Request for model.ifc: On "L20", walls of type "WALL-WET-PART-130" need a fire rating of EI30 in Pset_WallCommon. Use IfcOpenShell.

First a look at what the model holds.

```python
import ifcopenshell
import ifcopenshell.util.element

model = ifcopenshell.open("model.ifc")
print(model.schema)
storey = next(s for s in model.by_type("IfcBuildingStorey") if s.Name == "L20")
walls = [e for e in ifcopenshell.util.element.get_decomposition(storey) if e.is_a("IfcWall")]
seen = {}
for e in walls:
    element_type = ifcopenshell.util.element.get_type(e)
    key = (element_type.Name if element_type != e and element_type else None, ifcopenshell.util.element.get_pset(e, "Pset_WallCommon", "FireRating"))
    seen[key] = seen.get(key, 0) + 1
for (name, value), count in sorted(seen.items(), key=str):
    print(count, "x", name, "|", value)
```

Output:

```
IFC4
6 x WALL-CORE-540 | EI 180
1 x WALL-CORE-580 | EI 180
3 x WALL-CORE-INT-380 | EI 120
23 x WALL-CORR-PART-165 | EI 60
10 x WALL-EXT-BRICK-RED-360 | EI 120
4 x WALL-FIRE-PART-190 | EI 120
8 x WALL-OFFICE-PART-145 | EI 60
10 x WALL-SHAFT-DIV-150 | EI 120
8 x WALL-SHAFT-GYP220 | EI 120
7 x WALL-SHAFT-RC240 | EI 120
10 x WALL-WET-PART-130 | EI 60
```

```python
import ifcopenshell
import ifcopenshell.api.pset
import ifcopenshell.util.element

model = ifcopenshell.open("model.ifc")

storey = next(s for s in model.by_type("IfcBuildingStorey") if s.Name == "L20")
walls = [e for e in ifcopenshell.util.element.get_decomposition(storey) if e.is_a("IfcWall")]

count = 0
for e in walls:
    element_type = ifcopenshell.util.element.get_type(e)
    if element_type in (None, e) or element_type.Name != "WALL-WET-PART-130":
        continue
    found = ifcopenshell.util.element.get_pset(e, "Pset_WallCommon", should_inherit=False)
    if found:
        pset = model.by_id(found["id"])
        if len(ifcopenshell.util.element.get_elements_by_pset(pset)) > 1:
            pset = ifcopenshell.api.pset.unshare_pset(model, products=[e], pset=pset)[0]
    else:
        pset = ifcopenshell.api.pset.add_pset(model, product=e, name="Pset_WallCommon")
    ifcopenshell.api.pset.edit_pset(model, pset=pset, properties={"FireRating": "EI30"})
    count += 1

print(count, "walls updated")

model.write("model_updated.ifc")
```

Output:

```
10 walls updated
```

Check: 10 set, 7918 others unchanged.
